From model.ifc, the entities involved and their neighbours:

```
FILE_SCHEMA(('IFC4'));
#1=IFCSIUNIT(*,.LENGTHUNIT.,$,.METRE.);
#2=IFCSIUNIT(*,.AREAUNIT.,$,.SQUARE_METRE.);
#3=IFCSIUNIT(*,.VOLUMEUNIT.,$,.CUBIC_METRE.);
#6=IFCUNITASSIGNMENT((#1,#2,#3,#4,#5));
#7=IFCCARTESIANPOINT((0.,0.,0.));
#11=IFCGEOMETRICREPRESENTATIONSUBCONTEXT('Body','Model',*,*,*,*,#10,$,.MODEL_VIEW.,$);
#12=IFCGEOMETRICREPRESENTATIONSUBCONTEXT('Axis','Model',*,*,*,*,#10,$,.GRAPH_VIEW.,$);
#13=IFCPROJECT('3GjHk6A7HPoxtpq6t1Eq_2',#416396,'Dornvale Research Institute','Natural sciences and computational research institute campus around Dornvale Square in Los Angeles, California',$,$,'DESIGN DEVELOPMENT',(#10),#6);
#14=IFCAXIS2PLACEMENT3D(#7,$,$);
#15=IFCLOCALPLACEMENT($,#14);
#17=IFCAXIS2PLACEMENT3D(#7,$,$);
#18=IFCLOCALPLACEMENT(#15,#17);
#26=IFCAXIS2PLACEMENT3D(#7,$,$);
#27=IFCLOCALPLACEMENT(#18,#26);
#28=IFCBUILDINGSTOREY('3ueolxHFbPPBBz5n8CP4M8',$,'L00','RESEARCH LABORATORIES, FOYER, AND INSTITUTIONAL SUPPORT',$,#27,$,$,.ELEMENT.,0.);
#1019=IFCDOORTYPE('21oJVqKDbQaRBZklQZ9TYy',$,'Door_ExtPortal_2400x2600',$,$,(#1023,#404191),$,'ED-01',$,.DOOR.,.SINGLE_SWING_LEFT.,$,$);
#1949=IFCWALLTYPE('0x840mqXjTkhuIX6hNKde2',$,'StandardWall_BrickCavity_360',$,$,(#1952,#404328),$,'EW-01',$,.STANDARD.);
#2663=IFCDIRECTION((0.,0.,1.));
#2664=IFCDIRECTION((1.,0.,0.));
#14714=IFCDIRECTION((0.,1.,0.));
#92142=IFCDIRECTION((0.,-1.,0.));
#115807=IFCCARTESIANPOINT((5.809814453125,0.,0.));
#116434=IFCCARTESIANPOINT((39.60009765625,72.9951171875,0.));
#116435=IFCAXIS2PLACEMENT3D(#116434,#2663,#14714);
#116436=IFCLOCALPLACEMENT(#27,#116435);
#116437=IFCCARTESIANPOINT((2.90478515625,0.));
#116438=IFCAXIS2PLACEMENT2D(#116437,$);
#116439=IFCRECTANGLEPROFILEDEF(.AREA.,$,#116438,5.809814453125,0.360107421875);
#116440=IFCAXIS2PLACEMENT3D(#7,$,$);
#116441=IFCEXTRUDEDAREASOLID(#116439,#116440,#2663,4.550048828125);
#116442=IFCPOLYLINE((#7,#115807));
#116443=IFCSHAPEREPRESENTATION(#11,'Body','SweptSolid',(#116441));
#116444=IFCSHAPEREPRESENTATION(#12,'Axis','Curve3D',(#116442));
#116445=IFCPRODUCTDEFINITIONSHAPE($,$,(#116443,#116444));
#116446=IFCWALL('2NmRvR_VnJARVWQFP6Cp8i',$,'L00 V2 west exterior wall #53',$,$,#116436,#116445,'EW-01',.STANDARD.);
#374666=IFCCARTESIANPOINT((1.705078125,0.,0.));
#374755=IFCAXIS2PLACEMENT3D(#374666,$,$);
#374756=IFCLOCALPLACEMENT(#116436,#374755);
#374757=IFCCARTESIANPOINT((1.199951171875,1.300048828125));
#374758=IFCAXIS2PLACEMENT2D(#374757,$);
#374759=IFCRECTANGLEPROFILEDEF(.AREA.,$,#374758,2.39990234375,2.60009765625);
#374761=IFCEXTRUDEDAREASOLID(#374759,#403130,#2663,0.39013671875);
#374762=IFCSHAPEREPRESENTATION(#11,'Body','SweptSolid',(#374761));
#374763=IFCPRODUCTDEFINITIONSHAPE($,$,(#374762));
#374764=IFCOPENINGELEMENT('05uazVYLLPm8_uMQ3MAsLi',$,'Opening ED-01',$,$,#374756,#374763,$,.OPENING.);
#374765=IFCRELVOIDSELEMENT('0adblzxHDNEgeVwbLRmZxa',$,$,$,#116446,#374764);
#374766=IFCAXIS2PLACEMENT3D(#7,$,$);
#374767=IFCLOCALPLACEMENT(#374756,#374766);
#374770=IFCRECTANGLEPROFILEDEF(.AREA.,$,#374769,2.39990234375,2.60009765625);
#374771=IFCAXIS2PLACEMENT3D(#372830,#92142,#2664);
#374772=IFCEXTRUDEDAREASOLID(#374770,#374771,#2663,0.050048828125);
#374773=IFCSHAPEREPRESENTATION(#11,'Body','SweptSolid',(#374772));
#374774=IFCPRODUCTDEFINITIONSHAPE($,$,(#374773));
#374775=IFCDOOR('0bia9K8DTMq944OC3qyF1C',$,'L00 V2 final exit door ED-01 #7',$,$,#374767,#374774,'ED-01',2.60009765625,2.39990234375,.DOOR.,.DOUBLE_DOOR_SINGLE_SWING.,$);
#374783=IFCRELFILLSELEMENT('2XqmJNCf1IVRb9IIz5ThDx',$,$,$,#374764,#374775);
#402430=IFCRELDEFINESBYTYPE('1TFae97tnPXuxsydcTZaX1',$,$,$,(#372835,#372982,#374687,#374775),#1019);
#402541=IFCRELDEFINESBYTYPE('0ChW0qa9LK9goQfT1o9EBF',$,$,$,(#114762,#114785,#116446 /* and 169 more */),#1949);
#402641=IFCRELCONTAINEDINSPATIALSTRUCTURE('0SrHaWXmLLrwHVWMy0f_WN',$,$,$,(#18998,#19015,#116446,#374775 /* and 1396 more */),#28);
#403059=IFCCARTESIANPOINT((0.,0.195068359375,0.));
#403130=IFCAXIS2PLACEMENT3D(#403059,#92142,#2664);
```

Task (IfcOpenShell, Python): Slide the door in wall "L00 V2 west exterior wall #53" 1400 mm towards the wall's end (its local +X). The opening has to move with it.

```python
import ifcopenshell
import ifcopenshell.api.geometry
import ifcopenshell.util.placement

model = ifcopenshell.open("model.ifc")

door = model.by_guid("0bia9K8DTMq944OC3qyF1C")
opening = door.FillsVoids[0].RelatingOpeningElement
wall = opening.VoidsElements[0].RelatingBuildingElement

wall_matrix = ifcopenshell.util.placement.get_local_placement(wall.ObjectPlacement)
shift = wall_matrix[:3, 0] * 1.4
before = ifcopenshell.util.placement.get_local_placement(door.ObjectPlacement)[:3, 3].copy()

# The door is placed relative to its opening, so it follows when the opening moves.
matrix = ifcopenshell.util.placement.get_local_placement(opening.ObjectPlacement)
matrix[:3, 3] += shift
ifcopenshell.api.geometry.edit_object_placement(
    model, product=opening, matrix=matrix, is_si=False, should_transform_children=True
)

after = ifcopenshell.util.placement.get_local_placement(door.ObjectPlacement)[:3, 3]
print("door moved by", (after - before).round(3) + 0.0)

model.write("model_updated.ifc")
```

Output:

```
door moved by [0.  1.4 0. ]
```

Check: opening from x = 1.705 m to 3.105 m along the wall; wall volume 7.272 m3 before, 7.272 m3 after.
